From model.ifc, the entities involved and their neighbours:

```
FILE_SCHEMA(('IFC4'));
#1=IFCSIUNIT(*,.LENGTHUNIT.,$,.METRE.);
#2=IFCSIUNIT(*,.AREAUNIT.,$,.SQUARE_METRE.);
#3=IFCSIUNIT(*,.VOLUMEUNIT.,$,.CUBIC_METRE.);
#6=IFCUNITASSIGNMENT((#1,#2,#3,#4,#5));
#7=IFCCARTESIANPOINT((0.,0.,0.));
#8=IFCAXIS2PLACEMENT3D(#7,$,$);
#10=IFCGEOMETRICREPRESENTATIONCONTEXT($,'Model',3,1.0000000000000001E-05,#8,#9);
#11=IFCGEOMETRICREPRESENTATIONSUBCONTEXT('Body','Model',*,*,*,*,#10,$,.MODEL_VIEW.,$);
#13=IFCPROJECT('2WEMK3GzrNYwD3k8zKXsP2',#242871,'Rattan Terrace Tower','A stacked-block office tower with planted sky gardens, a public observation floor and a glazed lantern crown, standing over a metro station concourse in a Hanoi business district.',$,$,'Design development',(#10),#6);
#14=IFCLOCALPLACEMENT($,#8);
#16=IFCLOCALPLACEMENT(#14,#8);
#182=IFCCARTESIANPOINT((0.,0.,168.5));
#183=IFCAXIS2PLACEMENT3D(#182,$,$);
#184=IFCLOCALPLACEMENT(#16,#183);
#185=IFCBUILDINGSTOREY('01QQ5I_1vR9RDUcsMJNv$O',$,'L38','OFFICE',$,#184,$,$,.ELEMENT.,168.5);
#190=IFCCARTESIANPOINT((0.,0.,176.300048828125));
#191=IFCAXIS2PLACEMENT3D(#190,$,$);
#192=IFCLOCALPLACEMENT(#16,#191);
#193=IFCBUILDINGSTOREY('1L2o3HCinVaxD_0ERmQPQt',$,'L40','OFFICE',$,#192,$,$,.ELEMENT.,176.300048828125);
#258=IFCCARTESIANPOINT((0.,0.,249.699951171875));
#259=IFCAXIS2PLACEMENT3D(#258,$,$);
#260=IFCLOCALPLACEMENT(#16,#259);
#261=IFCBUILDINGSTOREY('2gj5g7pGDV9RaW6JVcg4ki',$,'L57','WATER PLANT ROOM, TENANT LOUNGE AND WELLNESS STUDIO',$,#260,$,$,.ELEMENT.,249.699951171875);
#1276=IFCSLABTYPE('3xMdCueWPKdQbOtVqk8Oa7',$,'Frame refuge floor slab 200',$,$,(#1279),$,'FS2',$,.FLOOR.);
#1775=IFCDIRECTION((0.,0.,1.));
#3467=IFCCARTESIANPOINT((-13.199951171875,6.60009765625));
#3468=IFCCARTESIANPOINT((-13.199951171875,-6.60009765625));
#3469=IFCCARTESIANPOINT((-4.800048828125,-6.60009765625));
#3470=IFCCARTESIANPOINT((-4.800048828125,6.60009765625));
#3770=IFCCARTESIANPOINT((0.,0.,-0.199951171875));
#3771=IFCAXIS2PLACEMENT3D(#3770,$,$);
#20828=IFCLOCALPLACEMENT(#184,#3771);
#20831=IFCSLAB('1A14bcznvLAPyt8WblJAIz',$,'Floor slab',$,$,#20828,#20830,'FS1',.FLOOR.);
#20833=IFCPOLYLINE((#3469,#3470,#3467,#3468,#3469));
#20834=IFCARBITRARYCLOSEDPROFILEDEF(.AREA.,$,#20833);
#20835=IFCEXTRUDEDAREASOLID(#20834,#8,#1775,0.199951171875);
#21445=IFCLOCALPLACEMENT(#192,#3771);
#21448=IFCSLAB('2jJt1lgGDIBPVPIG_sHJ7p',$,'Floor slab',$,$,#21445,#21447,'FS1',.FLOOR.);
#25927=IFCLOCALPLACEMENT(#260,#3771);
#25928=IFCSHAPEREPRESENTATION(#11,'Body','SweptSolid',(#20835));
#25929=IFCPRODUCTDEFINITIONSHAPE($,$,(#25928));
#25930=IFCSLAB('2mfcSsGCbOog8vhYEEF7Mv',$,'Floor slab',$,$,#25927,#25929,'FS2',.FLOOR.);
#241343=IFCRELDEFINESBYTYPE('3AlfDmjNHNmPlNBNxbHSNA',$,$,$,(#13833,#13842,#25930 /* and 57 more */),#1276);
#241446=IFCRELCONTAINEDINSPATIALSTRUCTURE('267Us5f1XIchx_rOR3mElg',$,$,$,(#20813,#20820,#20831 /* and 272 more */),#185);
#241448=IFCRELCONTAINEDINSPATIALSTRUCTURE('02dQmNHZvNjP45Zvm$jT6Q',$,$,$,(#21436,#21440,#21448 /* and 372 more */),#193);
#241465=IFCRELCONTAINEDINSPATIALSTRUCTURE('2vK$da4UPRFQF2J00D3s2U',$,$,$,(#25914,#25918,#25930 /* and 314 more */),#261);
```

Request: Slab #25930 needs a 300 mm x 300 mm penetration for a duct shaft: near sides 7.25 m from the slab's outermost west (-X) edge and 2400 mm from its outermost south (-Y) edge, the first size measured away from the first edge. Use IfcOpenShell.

```python
import numpy as np
import ifcopenshell
import ifcopenshell.api.feature
import ifcopenshell.api.geometry
import ifcopenshell.api.root
import ifcopenshell.geom
import ifcopenshell.util.placement
import ifcopenshell.util.representation
import ifcopenshell.util.shape
import ifcopenshell.util.unit

model = ifcopenshell.open("model.ifc")
unit_scale = ifcopenshell.util.unit.calculate_unit_scale(model)
settings = ifcopenshell.geom.settings()


def volume(element):
    """Net volume in cubic metres, openings subtracted."""
    shape = ifcopenshell.geom.create_shape(settings, element)
    return ifcopenshell.util.shape.get_volume(shape.geometry)


slab = model.by_guid("2mfcSsGCbOog8vhYEEF7Mv")
before = volume(slab)

# Extent in the slab's own axes, in metres. The edges named are its -X and -Y sides.
slab_shape = ifcopenshell.geom.create_shape(settings, slab)
vertices = ifcopenshell.util.shape.get_vertices(slab_shape.geometry)
x_min, y_min, bottom = vertices.min(axis=0)
top = vertices[:, 2].max()

opening = ifcopenshell.api.root.create_entity(model, ifc_class="IfcOpeningElement", name="Duct shaft opening", predefined_type="OPENING")
context = ifcopenshell.util.representation.get_context(model, "Model", "Body", "MODEL_VIEW")
width, depth = 0.3, 0.3
outline = [(0.0, 0.0), (width, 0.0), (width, depth), (0.0, depth), (0.0, 0.0)]
# Overshoot both faces by 50 mm so the cut is clean.
shape = ifcopenshell.api.geometry.add_slab_representation(
    model, context=context, depth=top - bottom + 0.1, polyline=outline
)
ifcopenshell.api.geometry.assign_representation(model, product=opening, representation=shape)

matrix = ifcopenshell.util.placement.get_local_placement(slab.ObjectPlacement)
matrix[:, 3] = matrix @ np.append(np.array([x_min + 7.25, y_min + 2.4, bottom - 0.05]) / unit_scale, 1.0)
ifcopenshell.api.geometry.edit_object_placement(model, product=opening, matrix=matrix, is_si=False)
ifcopenshell.api.feature.add_feature(model, feature=opening, element=slab)

after = volume(slab)

print(f"slab volume {before:.3f} -> {after:.3f} m3")

model.write("model_updated.ifc")
```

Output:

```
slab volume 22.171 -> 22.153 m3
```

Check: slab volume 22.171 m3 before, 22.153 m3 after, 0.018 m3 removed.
